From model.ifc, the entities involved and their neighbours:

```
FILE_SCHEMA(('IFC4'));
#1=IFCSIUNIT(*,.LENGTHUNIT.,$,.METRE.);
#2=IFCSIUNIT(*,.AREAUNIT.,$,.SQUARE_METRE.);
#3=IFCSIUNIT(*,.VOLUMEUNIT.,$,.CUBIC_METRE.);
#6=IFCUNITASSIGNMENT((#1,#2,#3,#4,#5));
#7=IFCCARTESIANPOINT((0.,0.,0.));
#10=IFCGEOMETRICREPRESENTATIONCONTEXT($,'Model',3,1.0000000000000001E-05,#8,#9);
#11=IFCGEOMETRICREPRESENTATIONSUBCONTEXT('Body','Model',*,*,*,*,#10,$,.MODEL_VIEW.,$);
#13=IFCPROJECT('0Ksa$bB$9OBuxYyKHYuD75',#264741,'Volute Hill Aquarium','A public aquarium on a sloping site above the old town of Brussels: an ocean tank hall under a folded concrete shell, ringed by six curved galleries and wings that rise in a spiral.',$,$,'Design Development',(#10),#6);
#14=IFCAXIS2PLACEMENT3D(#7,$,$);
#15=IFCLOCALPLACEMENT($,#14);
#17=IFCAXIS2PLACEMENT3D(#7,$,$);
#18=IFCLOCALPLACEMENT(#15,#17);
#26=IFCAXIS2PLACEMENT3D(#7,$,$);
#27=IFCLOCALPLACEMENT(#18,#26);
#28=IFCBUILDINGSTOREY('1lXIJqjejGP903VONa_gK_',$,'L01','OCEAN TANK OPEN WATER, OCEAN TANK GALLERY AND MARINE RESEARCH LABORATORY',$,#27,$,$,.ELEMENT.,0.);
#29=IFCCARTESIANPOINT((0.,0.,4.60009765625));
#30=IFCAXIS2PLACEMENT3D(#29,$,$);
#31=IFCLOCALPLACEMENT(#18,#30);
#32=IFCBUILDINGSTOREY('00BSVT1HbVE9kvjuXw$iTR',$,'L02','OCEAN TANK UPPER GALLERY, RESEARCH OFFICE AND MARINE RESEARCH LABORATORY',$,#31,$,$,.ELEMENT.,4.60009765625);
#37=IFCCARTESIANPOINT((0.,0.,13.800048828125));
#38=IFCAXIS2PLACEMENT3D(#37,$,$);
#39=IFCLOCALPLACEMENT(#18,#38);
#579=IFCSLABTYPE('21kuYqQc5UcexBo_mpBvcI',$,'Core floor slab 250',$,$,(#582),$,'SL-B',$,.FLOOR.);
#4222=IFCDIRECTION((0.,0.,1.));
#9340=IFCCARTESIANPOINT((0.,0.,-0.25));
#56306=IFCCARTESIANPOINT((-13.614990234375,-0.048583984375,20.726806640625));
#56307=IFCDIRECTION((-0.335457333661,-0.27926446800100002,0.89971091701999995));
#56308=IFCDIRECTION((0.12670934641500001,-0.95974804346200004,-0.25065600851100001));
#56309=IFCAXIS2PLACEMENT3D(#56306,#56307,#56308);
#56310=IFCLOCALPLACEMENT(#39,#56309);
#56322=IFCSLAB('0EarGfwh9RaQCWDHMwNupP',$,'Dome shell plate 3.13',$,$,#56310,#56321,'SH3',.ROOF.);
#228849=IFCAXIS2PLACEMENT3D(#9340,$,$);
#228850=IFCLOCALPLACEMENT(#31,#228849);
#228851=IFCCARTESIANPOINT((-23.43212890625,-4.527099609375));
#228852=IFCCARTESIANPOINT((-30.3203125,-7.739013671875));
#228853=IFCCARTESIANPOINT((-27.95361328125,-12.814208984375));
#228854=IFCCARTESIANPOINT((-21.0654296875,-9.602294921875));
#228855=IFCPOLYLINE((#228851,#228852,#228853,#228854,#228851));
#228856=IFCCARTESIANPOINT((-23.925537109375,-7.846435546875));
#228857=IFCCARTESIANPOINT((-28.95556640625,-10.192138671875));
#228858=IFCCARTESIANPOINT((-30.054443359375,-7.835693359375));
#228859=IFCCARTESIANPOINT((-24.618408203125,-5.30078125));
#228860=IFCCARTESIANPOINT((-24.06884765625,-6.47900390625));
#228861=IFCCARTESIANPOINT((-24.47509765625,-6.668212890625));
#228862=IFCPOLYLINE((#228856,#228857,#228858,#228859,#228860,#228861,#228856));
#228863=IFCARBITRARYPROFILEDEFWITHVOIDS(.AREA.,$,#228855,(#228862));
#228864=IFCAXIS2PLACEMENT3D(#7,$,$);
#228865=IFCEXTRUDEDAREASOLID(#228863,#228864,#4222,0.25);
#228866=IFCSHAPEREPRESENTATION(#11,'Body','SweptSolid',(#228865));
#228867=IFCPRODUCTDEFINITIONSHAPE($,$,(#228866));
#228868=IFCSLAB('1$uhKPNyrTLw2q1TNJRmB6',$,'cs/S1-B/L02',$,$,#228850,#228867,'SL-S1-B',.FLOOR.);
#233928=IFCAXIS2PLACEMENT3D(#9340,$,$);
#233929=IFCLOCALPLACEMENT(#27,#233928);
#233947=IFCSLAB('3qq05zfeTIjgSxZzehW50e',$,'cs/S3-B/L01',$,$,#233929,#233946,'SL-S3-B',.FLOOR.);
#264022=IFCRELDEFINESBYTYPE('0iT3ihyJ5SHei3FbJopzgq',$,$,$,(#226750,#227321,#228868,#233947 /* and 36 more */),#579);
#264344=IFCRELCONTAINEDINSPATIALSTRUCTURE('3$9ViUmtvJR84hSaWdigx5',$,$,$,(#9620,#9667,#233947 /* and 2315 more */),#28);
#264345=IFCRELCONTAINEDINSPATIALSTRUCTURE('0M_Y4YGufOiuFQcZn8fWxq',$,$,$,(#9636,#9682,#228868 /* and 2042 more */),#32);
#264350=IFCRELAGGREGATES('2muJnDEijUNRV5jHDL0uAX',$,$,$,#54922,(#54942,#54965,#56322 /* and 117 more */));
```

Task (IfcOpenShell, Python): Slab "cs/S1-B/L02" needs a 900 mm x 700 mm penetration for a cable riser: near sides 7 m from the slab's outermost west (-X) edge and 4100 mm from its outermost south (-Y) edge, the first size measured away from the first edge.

```python
import numpy as np
import ifcopenshell
import ifcopenshell.api.feature
import ifcopenshell.api.geometry
import ifcopenshell.api.root
import ifcopenshell.geom
import ifcopenshell.util.placement
import ifcopenshell.util.representation
import ifcopenshell.util.shape
import ifcopenshell.util.unit

model = ifcopenshell.open("model.ifc")
unit_scale = ifcopenshell.util.unit.calculate_unit_scale(model)
settings = ifcopenshell.geom.settings()


def volume(element):
    """Net volume in cubic metres, openings subtracted."""
    shape = ifcopenshell.geom.create_shape(settings, element)
    return ifcopenshell.util.shape.get_volume(shape.geometry)


slab = model.by_guid("1$uhKPNyrTLw2q1TNJRmB6")
before = volume(slab)

# Extent in the slab's own axes, in metres. The edges named are its -X and -Y sides.
slab_shape = ifcopenshell.geom.create_shape(settings, slab)
vertices = ifcopenshell.util.shape.get_vertices(slab_shape.geometry)
x_min, y_min, bottom = vertices.min(axis=0)
top = vertices[:, 2].max()

opening = ifcopenshell.api.root.create_entity(model, ifc_class="IfcOpeningElement", name="Cable riser opening", predefined_type="OPENING")
context = ifcopenshell.util.representation.get_context(model, "Model", "Body", "MODEL_VIEW")
width, depth = 0.9, 0.7
outline = [(0.0, 0.0), (width, 0.0), (width, depth), (0.0, depth), (0.0, 0.0)]
# Overshoot both faces by 50 mm so the cut is clean.
shape = ifcopenshell.api.geometry.add_slab_representation(
    model, context=context, depth=top - bottom + 0.1, polyline=outline
)
ifcopenshell.api.geometry.assign_representation(model, product=opening, representation=shape)

matrix = ifcopenshell.util.placement.get_local_placement(slab.ObjectPlacement)
matrix[:, 3] = matrix @ np.append(np.array([x_min + 7, y_min + 4.1, bottom - 0.05]) / unit_scale, 1.0)
ifcopenshell.api.geometry.edit_object_placement(model, product=opening, matrix=matrix, is_si=False)
ifcopenshell.api.feature.add_feature(model, feature=opening, element=slab)

after = volume(slab)

print(f"slab volume {before:.3f} -> {after:.3f} m3")

model.write("model_edited.ifc")
```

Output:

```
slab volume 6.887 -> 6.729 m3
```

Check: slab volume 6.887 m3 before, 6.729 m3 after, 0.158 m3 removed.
